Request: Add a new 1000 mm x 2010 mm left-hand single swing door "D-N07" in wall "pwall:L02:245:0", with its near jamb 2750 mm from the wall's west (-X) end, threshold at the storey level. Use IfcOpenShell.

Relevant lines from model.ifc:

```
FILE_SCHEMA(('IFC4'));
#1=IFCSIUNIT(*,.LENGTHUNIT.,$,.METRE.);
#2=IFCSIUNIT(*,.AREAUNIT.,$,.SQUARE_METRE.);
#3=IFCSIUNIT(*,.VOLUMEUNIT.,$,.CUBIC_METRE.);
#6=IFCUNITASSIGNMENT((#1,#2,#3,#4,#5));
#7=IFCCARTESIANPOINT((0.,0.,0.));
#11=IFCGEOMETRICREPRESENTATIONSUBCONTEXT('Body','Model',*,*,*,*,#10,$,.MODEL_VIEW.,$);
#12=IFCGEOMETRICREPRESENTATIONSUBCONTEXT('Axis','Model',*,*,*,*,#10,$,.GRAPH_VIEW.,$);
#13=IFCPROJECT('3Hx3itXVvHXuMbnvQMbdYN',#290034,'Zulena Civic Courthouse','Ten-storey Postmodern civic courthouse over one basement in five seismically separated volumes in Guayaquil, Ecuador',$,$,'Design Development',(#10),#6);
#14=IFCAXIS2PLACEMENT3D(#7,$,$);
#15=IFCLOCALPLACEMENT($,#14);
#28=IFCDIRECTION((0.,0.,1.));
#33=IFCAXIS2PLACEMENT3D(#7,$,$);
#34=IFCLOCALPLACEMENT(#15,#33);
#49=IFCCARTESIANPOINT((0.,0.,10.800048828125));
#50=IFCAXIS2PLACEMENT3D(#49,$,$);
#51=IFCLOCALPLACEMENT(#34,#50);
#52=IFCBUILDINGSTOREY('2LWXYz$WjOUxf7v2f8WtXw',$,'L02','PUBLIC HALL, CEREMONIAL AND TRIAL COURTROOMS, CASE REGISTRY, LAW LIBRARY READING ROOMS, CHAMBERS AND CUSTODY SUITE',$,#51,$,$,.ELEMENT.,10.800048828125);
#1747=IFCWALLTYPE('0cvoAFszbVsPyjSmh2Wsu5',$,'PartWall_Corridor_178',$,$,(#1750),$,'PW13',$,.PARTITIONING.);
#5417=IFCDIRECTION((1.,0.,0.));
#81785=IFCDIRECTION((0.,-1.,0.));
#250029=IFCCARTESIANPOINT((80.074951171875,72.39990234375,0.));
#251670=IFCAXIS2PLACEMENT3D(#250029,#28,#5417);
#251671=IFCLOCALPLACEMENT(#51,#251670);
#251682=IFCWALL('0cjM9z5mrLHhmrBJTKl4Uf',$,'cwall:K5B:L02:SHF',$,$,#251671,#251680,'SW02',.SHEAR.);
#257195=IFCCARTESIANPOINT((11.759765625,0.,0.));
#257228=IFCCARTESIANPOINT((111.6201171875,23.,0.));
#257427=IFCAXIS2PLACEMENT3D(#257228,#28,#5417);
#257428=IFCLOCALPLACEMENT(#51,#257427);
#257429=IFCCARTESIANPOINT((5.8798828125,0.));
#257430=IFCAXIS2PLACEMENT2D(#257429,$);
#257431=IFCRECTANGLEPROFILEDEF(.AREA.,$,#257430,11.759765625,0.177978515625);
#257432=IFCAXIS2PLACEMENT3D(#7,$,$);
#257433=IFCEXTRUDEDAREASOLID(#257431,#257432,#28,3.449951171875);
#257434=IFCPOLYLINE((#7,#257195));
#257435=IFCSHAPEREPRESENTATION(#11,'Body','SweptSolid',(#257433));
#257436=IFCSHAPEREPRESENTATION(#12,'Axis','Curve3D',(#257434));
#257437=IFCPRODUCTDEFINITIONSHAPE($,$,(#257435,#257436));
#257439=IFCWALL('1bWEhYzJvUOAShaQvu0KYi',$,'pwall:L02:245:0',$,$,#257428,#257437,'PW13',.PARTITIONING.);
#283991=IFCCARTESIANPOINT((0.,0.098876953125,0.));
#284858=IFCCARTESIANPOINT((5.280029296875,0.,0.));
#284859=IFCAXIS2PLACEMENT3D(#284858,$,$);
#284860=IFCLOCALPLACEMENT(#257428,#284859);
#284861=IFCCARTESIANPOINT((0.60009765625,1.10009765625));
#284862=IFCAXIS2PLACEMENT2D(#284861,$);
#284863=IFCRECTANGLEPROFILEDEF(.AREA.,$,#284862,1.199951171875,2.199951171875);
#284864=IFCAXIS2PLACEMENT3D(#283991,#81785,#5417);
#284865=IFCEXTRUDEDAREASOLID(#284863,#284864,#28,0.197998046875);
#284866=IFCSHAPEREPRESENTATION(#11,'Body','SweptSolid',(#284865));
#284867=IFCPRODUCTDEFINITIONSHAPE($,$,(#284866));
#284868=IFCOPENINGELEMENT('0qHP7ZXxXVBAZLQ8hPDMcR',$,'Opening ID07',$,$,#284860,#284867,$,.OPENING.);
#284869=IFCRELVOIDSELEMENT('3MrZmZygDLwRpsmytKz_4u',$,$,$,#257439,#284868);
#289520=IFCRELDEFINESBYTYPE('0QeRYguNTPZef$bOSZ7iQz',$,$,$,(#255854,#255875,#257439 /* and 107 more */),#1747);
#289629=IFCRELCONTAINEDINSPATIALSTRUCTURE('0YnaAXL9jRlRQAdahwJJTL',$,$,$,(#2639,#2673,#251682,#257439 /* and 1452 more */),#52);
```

```python
import numpy as np
import ifcopenshell
import ifcopenshell.api.feature
import ifcopenshell.api.geometry
import ifcopenshell.api.root
import ifcopenshell.api.spatial
import ifcopenshell.geom
import ifcopenshell.util.element
import ifcopenshell.util.placement
import ifcopenshell.util.representation
import ifcopenshell.util.shape
import ifcopenshell.util.unit

model = ifcopenshell.open("model.ifc")
unit_scale = ifcopenshell.util.unit.calculate_unit_scale(model)
settings = ifcopenshell.geom.settings()


def volume(element):
    """Net volume in cubic metres, openings subtracted."""
    shape = ifcopenshell.geom.create_shape(settings, element)
    return ifcopenshell.util.shape.get_volume(shape.geometry)


wall = model.by_id(257439)
storey = ifcopenshell.util.element.get_container(wall, ifc_class="IfcBuildingStorey")
context = ifcopenshell.util.representation.get_context(model, "Model", "Body", "MODEL_VIEW")
before = volume(wall)

width, height, from_end, sill = 1, 2.01, 2.75, 0.0  # metres

# The wall runs along its own X axis, and the end named is its -X end.
wall_shape = ifcopenshell.geom.create_shape(settings, wall)
x, y, z = ifcopenshell.util.shape.get_vertices(wall_shape.geometry).T
start = x.min() + from_end
face, thickness = float(y.min()), float(y.max() - y.min())
wall_matrix = ifcopenshell.util.placement.get_local_placement(wall.ObjectPlacement)
level = ifcopenshell.util.placement.get_local_placement(storey.ObjectPlacement)[2, 3]


def in_wall(x, y):
    """Placement at x, y metres in the wall's axes, at sill height."""
    matrix = wall_matrix.copy()
    matrix[:, 3] = wall_matrix @ np.array([x / unit_scale, y / unit_scale, 0.0, 1.0])
    matrix[2, 3] = level + sill / unit_scale
    return matrix


# Opening: a box that overshoots both wall faces by 50 mm.
opening = ifcopenshell.api.root.create_entity(model, ifc_class="IfcOpeningElement", predefined_type="OPENING")
box = ifcopenshell.api.geometry.add_wall_representation(
    model, context=context, length=width, height=height, thickness=thickness + 0.1
)
ifcopenshell.api.geometry.assign_representation(model, product=opening, representation=box)
ifcopenshell.api.geometry.edit_object_placement(model, product=opening, matrix=in_wall(start, face - 0.05), is_si=False)
ifcopenshell.api.feature.add_feature(model, feature=opening, element=wall)

door = ifcopenshell.api.root.create_entity(model, ifc_class="IfcDoor", name="D-N07", predefined_type="DOOR")
door.OverallWidth, door.OverallHeight = width / unit_scale, height / unit_scale
door.OperationType = "SINGLE_SWING_LEFT"
body = ifcopenshell.api.geometry.add_door_representation(
    model,
    context=context,
    overall_width=door.OverallWidth,
    overall_height=door.OverallHeight,
    operation_type="SINGLE_SWING_LEFT",
    lining_properties={"LiningDepth": thickness / unit_scale, "ThresholdDepth": thickness / unit_scale},
)
ifcopenshell.api.geometry.assign_representation(model, product=door, representation=body)
ifcopenshell.api.spatial.assign_container(model, products=[door], relating_structure=storey)
ifcopenshell.api.feature.add_filling(model, opening=opening, element=door)

# The lining spans the wall, so the door starts at the wall face.
ifcopenshell.api.geometry.edit_object_placement(model, product=door, matrix=in_wall(start, face), is_si=False)

after = volume(wall)

print(f"wall volume {before:.3f} -> {after:.3f} m3")

model.write("model_edited.ifc")
```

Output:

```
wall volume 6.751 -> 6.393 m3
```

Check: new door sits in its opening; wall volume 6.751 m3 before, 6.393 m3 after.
